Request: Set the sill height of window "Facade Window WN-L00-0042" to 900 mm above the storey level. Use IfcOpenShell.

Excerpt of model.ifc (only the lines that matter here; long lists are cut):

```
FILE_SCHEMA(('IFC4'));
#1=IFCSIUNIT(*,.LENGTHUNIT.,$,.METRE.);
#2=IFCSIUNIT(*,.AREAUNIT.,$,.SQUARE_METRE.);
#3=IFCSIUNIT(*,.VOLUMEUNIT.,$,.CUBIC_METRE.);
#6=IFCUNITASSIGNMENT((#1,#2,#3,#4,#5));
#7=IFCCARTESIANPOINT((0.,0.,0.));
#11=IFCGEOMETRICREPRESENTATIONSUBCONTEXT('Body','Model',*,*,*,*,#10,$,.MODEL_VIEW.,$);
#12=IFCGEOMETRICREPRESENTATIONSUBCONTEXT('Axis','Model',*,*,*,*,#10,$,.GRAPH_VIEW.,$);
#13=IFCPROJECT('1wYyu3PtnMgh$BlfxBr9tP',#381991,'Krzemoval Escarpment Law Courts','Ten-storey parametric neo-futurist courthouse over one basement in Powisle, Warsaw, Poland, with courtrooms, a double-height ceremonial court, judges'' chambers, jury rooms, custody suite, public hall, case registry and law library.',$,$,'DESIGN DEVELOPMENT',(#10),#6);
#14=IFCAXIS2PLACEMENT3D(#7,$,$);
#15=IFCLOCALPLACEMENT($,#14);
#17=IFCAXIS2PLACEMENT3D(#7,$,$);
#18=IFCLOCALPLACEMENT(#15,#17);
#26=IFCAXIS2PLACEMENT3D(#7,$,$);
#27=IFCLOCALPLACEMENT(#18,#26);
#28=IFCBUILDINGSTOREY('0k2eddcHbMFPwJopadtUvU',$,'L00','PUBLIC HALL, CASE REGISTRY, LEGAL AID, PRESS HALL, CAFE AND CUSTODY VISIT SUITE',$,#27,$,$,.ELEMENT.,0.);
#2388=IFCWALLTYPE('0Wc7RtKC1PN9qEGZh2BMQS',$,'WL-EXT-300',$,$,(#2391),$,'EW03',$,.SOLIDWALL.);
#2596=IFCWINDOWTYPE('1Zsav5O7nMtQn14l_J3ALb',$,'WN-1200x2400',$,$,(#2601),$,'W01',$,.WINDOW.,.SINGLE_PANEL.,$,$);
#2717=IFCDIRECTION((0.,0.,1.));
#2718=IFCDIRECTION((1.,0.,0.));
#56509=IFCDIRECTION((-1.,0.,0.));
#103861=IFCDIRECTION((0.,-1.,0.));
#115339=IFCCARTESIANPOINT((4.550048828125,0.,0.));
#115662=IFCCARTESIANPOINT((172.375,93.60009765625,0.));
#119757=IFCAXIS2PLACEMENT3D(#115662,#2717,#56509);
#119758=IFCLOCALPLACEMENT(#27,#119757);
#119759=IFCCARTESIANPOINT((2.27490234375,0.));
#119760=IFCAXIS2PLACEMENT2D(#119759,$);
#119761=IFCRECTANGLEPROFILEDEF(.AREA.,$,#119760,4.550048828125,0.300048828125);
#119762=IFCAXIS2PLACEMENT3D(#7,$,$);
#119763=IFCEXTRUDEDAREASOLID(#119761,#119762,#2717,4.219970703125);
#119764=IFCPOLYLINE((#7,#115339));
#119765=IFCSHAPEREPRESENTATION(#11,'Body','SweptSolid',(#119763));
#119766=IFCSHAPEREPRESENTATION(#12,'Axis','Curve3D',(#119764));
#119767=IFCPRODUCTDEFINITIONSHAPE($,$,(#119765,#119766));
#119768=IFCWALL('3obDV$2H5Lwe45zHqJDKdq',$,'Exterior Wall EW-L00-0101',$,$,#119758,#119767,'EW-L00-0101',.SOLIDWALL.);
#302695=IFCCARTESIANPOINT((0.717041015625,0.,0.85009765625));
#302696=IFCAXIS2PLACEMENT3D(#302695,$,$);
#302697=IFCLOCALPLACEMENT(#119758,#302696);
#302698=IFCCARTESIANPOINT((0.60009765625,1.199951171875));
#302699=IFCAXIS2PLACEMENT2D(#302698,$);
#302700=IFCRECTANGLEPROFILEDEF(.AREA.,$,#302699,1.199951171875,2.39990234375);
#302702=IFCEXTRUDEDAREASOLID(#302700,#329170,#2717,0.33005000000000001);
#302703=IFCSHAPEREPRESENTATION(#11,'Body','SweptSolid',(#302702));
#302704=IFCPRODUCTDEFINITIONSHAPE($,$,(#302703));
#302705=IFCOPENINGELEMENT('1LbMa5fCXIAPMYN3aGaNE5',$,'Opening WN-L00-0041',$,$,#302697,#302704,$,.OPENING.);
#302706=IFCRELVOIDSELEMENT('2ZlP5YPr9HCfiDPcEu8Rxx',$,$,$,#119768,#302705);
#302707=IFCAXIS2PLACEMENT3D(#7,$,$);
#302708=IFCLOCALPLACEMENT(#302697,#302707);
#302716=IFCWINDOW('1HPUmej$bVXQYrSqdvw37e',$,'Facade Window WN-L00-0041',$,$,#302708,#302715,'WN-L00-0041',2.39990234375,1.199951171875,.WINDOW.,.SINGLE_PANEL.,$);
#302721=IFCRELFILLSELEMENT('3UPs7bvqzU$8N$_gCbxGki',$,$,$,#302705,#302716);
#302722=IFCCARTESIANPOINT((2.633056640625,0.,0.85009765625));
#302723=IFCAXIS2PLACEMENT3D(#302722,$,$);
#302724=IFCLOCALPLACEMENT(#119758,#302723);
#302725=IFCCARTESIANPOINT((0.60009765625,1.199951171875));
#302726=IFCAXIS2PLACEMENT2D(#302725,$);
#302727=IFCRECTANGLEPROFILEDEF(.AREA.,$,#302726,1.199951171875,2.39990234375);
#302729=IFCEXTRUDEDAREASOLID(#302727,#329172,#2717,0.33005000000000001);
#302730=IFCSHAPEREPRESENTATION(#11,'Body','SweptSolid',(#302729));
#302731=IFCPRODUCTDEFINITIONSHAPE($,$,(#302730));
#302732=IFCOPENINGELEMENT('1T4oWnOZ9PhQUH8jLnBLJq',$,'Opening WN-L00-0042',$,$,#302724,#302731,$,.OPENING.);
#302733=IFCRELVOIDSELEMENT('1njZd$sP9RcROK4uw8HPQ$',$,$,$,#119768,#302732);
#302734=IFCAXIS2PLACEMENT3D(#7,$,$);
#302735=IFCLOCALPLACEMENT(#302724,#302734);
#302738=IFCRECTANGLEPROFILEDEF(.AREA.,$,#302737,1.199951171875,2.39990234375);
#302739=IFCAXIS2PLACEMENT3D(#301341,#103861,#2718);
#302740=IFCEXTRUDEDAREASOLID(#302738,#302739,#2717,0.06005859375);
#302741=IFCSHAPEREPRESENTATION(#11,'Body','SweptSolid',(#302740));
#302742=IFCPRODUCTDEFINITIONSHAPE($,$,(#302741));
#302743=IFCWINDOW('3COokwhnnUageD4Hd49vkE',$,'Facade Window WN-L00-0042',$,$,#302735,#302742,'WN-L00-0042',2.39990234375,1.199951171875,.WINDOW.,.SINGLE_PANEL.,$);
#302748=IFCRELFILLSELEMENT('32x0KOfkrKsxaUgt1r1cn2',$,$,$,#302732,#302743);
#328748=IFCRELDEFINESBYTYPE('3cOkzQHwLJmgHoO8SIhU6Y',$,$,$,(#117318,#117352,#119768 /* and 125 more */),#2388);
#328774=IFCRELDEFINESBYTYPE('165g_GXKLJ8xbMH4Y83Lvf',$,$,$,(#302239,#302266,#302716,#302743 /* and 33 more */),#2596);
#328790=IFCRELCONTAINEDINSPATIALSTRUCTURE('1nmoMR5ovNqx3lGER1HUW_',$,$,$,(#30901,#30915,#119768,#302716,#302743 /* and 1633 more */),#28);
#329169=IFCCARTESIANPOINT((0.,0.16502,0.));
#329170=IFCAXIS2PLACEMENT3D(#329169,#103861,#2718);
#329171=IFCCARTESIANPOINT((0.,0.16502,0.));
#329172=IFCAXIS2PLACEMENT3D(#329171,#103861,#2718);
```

```python
import numpy as np
import ifcopenshell
import ifcopenshell.api.geometry
import ifcopenshell.geom
import ifcopenshell.util.element
import ifcopenshell.util.placement
import ifcopenshell.util.shape
import ifcopenshell.util.unit

model = ifcopenshell.open("model.ifc")
unit_scale = ifcopenshell.util.unit.calculate_unit_scale(model)

window = model.by_guid("3COokwhnnUageD4Hd49vkE")
opening = window.FillsVoids[0].RelatingOpeningElement
storey = ifcopenshell.util.element.get_container(window, ifc_class="IfcBuildingStorey")
level = ifcopenshell.util.placement.get_local_placement(storey.ObjectPlacement)[2, 3]

# The opening's origin need not be at the sill, so measure its lowest point.
shape = ifcopenshell.geom.create_shape(ifcopenshell.geom.settings(), opening)
bottom = ifcopenshell.util.shape.get_shape_bottom_elevation(shape, shape.geometry) / unit_scale
dz = level + 0.9 / unit_scale - bottom

shift = np.array([0.0, 0.0, dz])
# The window is placed relative to its opening, so it follows when the opening moves.
matrix = ifcopenshell.util.placement.get_local_placement(opening.ObjectPlacement)
matrix[:3, 3] += shift
ifcopenshell.api.geometry.edit_object_placement(
    model, product=opening, matrix=matrix, is_si=False, should_transform_children=True
)

print(f"moved by {dz * unit_scale:+.3f} m")

model.write("model_edited.ifc")
```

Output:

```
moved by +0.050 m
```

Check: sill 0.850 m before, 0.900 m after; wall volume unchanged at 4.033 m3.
